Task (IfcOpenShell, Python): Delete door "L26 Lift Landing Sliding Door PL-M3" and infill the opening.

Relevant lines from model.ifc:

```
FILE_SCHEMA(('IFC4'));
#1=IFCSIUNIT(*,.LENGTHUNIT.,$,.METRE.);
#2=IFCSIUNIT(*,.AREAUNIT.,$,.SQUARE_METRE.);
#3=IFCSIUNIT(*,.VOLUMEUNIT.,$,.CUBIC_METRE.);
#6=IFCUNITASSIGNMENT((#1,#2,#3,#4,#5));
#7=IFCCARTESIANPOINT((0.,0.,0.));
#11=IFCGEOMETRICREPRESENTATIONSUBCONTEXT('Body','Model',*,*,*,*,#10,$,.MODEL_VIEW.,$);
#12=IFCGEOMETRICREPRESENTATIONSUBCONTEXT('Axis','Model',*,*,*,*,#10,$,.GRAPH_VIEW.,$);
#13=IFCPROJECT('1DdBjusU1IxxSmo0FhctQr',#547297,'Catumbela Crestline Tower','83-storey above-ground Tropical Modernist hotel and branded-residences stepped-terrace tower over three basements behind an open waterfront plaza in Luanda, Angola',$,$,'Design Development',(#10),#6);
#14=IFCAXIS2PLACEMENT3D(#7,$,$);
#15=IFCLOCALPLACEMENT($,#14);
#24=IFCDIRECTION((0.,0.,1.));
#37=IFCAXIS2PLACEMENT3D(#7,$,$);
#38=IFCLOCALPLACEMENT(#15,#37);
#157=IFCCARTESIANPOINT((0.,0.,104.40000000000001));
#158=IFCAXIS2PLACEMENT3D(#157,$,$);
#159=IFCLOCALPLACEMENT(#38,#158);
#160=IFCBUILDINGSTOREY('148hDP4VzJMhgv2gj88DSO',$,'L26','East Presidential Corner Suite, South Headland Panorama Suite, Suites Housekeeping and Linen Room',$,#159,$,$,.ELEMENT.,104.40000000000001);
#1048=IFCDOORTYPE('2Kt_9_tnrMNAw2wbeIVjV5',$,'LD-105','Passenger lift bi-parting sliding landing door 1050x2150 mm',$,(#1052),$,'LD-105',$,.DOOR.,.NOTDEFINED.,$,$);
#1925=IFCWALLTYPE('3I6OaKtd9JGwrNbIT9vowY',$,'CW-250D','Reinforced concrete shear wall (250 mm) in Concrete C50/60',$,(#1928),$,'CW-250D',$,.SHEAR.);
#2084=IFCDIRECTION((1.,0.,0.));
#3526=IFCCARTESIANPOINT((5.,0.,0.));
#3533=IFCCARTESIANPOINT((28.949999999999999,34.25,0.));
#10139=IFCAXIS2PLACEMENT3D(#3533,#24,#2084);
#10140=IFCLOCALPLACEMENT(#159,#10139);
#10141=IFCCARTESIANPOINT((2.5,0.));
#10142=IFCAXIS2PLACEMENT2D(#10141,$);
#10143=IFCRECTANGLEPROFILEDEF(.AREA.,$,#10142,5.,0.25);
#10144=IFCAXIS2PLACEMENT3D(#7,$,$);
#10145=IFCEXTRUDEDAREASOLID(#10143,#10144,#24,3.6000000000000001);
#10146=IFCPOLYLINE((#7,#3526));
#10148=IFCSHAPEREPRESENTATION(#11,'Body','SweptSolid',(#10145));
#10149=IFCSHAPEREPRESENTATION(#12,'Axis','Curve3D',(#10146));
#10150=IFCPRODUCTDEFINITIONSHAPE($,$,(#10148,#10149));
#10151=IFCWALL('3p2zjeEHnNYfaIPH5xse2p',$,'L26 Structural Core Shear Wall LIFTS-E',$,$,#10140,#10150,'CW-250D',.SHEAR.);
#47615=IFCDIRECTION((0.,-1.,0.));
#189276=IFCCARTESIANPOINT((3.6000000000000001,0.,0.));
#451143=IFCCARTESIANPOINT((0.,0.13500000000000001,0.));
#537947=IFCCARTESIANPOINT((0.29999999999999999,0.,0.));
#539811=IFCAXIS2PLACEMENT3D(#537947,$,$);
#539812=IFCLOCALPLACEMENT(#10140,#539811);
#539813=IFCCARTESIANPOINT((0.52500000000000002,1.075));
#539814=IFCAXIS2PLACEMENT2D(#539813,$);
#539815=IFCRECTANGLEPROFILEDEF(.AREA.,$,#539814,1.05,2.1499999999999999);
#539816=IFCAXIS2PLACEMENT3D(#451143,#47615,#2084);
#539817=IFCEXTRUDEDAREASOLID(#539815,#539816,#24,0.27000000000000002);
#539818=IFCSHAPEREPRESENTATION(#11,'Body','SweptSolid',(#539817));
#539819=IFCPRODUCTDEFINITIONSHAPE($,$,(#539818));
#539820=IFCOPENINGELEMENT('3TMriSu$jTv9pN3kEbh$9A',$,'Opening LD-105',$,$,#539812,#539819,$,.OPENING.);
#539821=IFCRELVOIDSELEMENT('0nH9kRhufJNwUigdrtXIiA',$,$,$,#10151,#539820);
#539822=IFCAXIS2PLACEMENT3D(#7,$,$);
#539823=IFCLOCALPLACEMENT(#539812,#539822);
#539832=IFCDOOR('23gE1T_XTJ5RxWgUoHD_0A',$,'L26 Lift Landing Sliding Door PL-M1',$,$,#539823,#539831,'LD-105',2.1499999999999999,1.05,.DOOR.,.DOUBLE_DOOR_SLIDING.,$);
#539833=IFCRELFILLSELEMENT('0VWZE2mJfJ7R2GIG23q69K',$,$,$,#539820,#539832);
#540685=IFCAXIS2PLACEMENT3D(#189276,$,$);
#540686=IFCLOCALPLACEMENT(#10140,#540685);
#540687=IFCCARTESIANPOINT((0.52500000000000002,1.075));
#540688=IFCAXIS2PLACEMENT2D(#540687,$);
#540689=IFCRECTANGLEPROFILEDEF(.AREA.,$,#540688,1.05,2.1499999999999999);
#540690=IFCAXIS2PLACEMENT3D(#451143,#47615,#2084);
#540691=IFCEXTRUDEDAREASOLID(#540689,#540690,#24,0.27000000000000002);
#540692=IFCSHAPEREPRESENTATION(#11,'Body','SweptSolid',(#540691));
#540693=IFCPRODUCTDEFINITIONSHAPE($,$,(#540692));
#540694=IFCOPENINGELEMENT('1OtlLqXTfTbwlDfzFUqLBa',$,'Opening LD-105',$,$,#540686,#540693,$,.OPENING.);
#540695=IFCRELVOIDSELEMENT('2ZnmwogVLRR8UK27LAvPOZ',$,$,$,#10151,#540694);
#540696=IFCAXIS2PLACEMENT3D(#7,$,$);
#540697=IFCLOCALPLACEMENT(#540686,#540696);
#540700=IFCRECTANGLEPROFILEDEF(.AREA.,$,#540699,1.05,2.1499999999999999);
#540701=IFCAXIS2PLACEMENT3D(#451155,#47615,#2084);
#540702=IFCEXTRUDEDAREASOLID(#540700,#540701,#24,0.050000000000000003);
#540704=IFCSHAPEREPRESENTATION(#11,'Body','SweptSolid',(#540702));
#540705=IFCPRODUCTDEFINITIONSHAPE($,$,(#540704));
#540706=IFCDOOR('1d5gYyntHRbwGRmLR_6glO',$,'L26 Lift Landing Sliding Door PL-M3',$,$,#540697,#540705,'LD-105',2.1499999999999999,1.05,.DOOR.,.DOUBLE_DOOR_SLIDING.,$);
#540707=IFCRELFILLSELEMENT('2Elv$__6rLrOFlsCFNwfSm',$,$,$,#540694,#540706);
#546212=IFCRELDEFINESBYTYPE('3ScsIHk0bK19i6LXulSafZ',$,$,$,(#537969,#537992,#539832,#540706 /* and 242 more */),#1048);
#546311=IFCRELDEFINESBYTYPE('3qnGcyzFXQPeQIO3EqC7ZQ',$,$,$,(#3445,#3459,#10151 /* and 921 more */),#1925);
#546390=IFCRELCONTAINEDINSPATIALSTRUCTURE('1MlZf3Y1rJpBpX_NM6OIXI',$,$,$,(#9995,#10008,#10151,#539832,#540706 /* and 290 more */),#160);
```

```python
import ifcopenshell
import ifcopenshell.api.feature
import ifcopenshell.api.root
import ifcopenshell.geom
import ifcopenshell.util.shape

model = ifcopenshell.open("model.ifc")
settings = ifcopenshell.geom.settings()


def volume(element):
    """Net volume in cubic metres, openings subtracted."""
    shape = ifcopenshell.geom.create_shape(settings, element)
    return ifcopenshell.util.shape.get_volume(shape.geometry)


door = model.by_guid("1d5gYyntHRbwGRmLR_6glO")
opening = door.FillsVoids[0].RelatingOpeningElement
wall = opening.VoidsElements[0].RelatingBuildingElement
before = volume(wall)

ifcopenshell.api.root.remove_product(model, product=door)
ifcopenshell.api.feature.remove_feature(model, feature=opening)

after = volume(wall)

print(f"wall volume {before:.3f} -> {after:.3f} m3")

model.write("model_v2.ifc")
```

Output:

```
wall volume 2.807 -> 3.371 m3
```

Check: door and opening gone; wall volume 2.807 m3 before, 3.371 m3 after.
